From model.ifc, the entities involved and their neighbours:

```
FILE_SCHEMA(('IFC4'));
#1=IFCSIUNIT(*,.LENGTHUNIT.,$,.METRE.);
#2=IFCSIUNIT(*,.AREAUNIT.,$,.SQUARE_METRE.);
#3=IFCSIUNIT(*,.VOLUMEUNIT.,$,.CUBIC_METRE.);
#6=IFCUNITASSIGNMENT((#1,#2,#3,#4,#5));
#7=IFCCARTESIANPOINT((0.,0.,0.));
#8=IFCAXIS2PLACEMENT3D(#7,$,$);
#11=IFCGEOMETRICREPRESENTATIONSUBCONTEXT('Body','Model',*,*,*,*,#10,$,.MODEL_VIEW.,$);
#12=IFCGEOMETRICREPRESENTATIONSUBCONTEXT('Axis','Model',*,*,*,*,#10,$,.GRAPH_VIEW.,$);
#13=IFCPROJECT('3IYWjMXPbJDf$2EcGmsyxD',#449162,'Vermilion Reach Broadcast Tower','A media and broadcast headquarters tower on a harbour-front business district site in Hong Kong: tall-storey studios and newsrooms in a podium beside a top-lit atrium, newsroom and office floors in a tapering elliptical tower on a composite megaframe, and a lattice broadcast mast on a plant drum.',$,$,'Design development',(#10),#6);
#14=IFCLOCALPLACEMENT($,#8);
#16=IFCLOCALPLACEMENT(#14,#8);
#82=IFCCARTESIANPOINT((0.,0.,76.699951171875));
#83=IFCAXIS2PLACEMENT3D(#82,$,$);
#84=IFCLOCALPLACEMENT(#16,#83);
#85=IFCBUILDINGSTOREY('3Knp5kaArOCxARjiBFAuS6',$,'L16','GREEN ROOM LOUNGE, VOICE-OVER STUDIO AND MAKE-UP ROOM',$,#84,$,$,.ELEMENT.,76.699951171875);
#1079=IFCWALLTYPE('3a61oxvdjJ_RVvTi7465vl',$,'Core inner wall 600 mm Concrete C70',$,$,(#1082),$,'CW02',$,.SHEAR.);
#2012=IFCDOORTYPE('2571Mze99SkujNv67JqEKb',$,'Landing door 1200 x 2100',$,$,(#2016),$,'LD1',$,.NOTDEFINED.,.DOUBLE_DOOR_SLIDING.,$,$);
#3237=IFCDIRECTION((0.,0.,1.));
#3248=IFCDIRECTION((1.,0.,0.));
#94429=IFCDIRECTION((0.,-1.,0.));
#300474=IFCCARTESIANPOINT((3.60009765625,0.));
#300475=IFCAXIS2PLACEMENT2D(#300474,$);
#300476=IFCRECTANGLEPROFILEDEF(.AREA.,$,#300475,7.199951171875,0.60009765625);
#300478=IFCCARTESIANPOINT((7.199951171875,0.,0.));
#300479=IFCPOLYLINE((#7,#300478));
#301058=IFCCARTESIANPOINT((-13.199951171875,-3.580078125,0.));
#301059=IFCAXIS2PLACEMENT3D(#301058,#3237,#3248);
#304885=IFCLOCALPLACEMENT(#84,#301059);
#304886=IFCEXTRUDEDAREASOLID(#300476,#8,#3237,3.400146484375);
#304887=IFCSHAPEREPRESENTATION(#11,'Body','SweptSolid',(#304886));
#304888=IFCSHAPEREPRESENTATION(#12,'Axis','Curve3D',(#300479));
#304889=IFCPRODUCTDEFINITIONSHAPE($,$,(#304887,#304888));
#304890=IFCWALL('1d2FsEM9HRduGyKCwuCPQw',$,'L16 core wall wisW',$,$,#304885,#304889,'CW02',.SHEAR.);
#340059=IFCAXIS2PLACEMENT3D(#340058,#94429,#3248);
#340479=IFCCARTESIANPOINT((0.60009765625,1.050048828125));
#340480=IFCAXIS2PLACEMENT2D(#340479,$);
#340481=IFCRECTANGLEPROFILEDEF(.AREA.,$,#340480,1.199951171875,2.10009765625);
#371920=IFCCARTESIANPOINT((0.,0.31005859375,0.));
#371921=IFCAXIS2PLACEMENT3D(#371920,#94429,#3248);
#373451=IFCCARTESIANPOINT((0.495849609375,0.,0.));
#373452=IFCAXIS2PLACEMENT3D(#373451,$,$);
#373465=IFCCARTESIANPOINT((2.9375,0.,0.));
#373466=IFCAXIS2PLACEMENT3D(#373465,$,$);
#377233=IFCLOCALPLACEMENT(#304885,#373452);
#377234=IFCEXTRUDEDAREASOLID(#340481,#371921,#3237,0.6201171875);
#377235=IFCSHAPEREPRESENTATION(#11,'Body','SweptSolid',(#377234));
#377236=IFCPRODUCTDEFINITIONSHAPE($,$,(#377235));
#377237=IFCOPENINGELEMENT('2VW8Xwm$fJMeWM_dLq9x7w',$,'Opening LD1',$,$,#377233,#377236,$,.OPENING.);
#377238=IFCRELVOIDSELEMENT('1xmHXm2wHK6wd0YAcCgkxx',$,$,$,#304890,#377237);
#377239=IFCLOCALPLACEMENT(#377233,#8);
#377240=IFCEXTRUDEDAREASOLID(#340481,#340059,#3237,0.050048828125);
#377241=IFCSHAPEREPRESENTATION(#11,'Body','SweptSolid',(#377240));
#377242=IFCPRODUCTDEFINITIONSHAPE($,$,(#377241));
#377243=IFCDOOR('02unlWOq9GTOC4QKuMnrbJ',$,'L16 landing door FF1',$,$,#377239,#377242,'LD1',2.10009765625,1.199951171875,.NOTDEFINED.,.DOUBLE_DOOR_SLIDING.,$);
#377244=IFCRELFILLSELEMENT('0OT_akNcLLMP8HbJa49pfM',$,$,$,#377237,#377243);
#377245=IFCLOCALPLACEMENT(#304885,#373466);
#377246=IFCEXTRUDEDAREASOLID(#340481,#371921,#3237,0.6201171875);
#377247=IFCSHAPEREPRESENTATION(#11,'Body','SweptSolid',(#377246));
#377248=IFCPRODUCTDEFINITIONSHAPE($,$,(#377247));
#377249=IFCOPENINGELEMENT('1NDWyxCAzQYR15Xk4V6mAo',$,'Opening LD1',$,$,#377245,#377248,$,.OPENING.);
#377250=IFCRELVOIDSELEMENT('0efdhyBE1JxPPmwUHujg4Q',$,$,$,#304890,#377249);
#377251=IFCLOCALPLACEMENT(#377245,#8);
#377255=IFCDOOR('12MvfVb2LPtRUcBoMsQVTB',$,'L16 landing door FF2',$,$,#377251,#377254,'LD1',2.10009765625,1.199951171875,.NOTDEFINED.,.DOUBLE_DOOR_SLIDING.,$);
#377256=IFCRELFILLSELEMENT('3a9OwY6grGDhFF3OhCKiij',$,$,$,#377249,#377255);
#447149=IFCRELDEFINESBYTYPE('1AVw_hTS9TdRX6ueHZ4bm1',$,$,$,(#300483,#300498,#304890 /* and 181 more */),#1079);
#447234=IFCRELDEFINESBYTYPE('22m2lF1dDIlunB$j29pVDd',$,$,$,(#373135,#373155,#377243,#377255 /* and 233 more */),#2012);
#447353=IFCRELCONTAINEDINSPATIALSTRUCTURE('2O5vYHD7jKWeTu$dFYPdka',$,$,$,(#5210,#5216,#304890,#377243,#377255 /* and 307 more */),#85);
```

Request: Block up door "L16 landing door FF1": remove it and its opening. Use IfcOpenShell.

```python
import ifcopenshell
import ifcopenshell.api.feature
import ifcopenshell.api.root
import ifcopenshell.geom
import ifcopenshell.util.shape

model = ifcopenshell.open("model.ifc")
settings = ifcopenshell.geom.settings()


def volume(element):
    """Net volume in cubic metres, openings subtracted."""
    shape = ifcopenshell.geom.create_shape(settings, element)
    return ifcopenshell.util.shape.get_volume(shape.geometry)


door = model.by_guid("02unlWOq9GTOC4QKuMnrbJ")
opening = door.FillsVoids[0].RelatingOpeningElement
wall = opening.VoidsElements[0].RelatingBuildingElement
before = volume(wall)

ifcopenshell.api.root.remove_product(model, product=door)
ifcopenshell.api.feature.remove_feature(model, feature=opening)

after = volume(wall)

print(f"wall volume {before:.3f} -> {after:.3f} m3")

model.write("model_updated.ifc")
```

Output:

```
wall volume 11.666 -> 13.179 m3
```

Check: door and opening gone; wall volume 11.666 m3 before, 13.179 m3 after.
